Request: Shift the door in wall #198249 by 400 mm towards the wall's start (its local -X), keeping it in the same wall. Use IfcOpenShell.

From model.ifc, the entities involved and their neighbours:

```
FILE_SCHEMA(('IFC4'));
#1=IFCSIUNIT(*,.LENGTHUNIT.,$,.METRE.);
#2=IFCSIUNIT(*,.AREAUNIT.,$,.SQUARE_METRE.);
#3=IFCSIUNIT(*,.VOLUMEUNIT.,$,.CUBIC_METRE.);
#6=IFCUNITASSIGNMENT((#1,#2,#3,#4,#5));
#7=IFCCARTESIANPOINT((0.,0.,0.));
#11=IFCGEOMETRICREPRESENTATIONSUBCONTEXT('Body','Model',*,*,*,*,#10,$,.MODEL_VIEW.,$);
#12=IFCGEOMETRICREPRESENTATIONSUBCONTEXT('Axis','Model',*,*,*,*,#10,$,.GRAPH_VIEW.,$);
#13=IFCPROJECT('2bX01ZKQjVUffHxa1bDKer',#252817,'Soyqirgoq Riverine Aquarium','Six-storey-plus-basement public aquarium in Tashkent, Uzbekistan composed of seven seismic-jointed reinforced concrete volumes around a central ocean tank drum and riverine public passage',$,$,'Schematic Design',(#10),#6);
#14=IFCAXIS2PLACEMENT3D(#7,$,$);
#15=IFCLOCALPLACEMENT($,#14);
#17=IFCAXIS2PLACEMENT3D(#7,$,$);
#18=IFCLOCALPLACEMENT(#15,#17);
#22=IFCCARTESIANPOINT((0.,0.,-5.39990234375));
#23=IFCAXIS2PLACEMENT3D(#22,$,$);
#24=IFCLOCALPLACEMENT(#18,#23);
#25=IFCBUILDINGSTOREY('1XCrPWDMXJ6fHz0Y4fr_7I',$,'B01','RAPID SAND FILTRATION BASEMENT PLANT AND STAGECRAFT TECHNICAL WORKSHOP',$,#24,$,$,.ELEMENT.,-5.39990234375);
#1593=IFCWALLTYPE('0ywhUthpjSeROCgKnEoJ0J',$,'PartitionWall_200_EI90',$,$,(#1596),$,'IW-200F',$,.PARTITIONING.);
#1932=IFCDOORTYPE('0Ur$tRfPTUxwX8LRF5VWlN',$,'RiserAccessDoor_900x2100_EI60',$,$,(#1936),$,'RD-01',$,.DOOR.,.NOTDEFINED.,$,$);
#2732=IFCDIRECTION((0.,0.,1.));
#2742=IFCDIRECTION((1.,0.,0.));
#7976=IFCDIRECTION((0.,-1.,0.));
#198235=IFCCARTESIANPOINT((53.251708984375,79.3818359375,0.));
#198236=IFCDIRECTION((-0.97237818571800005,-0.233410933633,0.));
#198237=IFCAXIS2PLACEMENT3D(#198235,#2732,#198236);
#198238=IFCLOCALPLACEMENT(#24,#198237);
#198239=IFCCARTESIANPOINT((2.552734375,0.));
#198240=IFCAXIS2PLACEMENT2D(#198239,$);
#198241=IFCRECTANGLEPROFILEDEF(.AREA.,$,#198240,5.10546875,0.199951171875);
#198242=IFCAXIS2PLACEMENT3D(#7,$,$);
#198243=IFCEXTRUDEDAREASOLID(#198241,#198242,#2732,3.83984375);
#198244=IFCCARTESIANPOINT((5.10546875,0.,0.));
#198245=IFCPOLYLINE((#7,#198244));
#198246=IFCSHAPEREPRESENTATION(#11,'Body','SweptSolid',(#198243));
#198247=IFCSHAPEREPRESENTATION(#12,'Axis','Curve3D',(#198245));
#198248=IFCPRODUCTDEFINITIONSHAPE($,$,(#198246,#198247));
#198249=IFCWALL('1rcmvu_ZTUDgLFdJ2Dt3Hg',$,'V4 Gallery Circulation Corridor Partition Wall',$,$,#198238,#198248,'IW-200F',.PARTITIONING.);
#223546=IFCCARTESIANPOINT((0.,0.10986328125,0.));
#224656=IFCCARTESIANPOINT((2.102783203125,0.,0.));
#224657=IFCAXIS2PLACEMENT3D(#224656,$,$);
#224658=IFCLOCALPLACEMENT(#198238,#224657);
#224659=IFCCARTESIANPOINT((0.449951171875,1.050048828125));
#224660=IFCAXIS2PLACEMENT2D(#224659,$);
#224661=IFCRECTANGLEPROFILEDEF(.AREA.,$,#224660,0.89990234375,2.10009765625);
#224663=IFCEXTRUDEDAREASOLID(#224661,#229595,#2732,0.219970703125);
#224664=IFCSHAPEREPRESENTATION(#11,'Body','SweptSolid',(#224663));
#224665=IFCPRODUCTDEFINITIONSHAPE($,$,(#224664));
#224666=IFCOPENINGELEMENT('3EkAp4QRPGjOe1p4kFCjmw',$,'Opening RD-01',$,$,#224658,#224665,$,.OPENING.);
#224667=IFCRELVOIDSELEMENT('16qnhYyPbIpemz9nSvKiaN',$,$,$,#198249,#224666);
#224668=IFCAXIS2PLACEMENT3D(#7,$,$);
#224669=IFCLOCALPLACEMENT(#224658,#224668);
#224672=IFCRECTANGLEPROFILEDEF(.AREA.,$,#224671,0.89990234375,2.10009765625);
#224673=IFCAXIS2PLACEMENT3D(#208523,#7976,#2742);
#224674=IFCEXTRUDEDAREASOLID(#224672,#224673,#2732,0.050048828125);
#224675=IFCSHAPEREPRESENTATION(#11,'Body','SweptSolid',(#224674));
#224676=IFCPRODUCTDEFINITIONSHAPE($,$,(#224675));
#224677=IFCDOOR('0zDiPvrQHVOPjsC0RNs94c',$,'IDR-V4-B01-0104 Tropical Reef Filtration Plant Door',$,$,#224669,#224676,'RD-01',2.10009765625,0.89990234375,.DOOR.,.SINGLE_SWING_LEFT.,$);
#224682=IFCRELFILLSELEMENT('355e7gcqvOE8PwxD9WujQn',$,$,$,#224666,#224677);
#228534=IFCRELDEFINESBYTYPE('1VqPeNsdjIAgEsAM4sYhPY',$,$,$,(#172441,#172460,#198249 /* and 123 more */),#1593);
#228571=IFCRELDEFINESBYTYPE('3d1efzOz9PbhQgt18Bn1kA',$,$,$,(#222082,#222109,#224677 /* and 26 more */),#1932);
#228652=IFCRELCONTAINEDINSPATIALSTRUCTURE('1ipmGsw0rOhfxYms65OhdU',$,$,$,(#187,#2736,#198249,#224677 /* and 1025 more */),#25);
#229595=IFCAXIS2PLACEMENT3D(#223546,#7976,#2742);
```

```python
import ifcopenshell
import ifcopenshell.api.geometry
import ifcopenshell.util.placement

model = ifcopenshell.open("model.ifc")

door = model.by_guid("0zDiPvrQHVOPjsC0RNs94c")
opening = door.FillsVoids[0].RelatingOpeningElement
wall = opening.VoidsElements[0].RelatingBuildingElement

wall_matrix = ifcopenshell.util.placement.get_local_placement(wall.ObjectPlacement)
shift = wall_matrix[:3, 0] * -0.4
before = ifcopenshell.util.placement.get_local_placement(door.ObjectPlacement)[:3, 3].copy()

# The door is placed relative to its opening, so it follows when the opening moves.
matrix = ifcopenshell.util.placement.get_local_placement(opening.ObjectPlacement)
matrix[:3, 3] += shift
ifcopenshell.api.geometry.edit_object_placement(
    model, product=opening, matrix=matrix, is_si=False, should_transform_children=True
)

after = ifcopenshell.util.placement.get_local_placement(door.ObjectPlacement)[:3, 3]
print("door moved by", (after - before).round(3) + 0.0)

model.write("model-out.ifc")
```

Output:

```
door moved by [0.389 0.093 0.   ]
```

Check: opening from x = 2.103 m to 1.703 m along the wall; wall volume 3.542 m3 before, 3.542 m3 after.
